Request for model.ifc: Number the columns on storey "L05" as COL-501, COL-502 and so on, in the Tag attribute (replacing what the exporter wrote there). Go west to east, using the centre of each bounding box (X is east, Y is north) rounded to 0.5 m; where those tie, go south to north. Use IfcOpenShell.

First a look at what the model holds.

```python
import ifcopenshell
import ifcopenshell.util.element
import ifcopenshell.util.placement

model = ifcopenshell.open("model.ifc")
print(model.schema)
storey = next(s for s in model.by_type("IfcBuildingStorey") if s.Name == "L05")
columns = [e for e in ifcopenshell.util.element.get_decomposition(storey) if e.is_a("IfcColumn")]
for e in sorted(columns, key=lambda e: e.id()):
    origin = ifcopenshell.util.placement.get_local_placement(e.ObjectPlacement)[:3, 3]
    print(e.id(), e.Tag, e.Name, origin.round(2) + 0.0, sep=" | ")
```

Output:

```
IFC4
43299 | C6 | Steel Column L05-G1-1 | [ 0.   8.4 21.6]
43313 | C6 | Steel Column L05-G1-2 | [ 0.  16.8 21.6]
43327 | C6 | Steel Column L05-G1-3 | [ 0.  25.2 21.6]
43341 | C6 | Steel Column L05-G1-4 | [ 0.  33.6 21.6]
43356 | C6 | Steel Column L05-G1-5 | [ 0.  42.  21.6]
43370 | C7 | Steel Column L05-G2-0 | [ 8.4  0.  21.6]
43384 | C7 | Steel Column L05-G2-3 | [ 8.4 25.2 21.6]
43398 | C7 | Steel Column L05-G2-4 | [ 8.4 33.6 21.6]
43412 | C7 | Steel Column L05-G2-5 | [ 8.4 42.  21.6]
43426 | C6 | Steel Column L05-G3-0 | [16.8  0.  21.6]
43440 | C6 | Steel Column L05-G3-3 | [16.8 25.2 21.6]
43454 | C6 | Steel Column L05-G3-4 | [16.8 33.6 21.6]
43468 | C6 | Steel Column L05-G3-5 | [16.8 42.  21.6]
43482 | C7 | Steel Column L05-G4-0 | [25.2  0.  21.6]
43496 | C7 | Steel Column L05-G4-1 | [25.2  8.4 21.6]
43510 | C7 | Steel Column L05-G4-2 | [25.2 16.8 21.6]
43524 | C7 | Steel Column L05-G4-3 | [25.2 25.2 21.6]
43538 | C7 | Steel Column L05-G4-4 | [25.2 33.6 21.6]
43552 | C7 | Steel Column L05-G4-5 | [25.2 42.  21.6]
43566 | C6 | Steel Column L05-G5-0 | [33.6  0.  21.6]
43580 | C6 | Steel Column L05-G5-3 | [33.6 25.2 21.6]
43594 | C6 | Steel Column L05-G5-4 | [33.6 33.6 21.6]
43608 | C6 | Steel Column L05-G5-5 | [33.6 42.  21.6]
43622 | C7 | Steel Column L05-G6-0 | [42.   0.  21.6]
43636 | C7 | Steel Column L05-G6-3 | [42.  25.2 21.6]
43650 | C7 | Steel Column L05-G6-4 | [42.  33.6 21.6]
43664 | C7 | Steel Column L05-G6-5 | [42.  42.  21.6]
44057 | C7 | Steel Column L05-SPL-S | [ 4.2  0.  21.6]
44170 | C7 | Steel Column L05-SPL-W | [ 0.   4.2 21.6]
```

```python
import ifcopenshell
import ifcopenshell.geom
import ifcopenshell.util.element
import ifcopenshell.util.shape

model = ifcopenshell.open("model.ifc")
settings = ifcopenshell.geom.settings()
settings.set("use-world-coords", True)


def centre(element):
    shape = ifcopenshell.geom.create_shape(settings, element)
    return ifcopenshell.util.shape.get_bbox_centroid(shape.geometry)


storey = next(s for s in model.by_type("IfcBuildingStorey") if s.Name == "L05")
columns = [e for e in ifcopenshell.util.element.get_decomposition(storey) if e.is_a("IfcColumn")]

# Insertion points can sit at a corner or the storey origin, so sort by the geometry (in metres).
centres = {e: centre(e) for e in columns}
columns.sort(key=lambda e: (round(centres[e][0] / 0.5), centres[e][1]))

for i, e in enumerate(columns, start=1):
    number = f"COL-5{i:02d}"
    e.Tag = number
    print(e.id(), number)

model.write("model_rev.ifc")
```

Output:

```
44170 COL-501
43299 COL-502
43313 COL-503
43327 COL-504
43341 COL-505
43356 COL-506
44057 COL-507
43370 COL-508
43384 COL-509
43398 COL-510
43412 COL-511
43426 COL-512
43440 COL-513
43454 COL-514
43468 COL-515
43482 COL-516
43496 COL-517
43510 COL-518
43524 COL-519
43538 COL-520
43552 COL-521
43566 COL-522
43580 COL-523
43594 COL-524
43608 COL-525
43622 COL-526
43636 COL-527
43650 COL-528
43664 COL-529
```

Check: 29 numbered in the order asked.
